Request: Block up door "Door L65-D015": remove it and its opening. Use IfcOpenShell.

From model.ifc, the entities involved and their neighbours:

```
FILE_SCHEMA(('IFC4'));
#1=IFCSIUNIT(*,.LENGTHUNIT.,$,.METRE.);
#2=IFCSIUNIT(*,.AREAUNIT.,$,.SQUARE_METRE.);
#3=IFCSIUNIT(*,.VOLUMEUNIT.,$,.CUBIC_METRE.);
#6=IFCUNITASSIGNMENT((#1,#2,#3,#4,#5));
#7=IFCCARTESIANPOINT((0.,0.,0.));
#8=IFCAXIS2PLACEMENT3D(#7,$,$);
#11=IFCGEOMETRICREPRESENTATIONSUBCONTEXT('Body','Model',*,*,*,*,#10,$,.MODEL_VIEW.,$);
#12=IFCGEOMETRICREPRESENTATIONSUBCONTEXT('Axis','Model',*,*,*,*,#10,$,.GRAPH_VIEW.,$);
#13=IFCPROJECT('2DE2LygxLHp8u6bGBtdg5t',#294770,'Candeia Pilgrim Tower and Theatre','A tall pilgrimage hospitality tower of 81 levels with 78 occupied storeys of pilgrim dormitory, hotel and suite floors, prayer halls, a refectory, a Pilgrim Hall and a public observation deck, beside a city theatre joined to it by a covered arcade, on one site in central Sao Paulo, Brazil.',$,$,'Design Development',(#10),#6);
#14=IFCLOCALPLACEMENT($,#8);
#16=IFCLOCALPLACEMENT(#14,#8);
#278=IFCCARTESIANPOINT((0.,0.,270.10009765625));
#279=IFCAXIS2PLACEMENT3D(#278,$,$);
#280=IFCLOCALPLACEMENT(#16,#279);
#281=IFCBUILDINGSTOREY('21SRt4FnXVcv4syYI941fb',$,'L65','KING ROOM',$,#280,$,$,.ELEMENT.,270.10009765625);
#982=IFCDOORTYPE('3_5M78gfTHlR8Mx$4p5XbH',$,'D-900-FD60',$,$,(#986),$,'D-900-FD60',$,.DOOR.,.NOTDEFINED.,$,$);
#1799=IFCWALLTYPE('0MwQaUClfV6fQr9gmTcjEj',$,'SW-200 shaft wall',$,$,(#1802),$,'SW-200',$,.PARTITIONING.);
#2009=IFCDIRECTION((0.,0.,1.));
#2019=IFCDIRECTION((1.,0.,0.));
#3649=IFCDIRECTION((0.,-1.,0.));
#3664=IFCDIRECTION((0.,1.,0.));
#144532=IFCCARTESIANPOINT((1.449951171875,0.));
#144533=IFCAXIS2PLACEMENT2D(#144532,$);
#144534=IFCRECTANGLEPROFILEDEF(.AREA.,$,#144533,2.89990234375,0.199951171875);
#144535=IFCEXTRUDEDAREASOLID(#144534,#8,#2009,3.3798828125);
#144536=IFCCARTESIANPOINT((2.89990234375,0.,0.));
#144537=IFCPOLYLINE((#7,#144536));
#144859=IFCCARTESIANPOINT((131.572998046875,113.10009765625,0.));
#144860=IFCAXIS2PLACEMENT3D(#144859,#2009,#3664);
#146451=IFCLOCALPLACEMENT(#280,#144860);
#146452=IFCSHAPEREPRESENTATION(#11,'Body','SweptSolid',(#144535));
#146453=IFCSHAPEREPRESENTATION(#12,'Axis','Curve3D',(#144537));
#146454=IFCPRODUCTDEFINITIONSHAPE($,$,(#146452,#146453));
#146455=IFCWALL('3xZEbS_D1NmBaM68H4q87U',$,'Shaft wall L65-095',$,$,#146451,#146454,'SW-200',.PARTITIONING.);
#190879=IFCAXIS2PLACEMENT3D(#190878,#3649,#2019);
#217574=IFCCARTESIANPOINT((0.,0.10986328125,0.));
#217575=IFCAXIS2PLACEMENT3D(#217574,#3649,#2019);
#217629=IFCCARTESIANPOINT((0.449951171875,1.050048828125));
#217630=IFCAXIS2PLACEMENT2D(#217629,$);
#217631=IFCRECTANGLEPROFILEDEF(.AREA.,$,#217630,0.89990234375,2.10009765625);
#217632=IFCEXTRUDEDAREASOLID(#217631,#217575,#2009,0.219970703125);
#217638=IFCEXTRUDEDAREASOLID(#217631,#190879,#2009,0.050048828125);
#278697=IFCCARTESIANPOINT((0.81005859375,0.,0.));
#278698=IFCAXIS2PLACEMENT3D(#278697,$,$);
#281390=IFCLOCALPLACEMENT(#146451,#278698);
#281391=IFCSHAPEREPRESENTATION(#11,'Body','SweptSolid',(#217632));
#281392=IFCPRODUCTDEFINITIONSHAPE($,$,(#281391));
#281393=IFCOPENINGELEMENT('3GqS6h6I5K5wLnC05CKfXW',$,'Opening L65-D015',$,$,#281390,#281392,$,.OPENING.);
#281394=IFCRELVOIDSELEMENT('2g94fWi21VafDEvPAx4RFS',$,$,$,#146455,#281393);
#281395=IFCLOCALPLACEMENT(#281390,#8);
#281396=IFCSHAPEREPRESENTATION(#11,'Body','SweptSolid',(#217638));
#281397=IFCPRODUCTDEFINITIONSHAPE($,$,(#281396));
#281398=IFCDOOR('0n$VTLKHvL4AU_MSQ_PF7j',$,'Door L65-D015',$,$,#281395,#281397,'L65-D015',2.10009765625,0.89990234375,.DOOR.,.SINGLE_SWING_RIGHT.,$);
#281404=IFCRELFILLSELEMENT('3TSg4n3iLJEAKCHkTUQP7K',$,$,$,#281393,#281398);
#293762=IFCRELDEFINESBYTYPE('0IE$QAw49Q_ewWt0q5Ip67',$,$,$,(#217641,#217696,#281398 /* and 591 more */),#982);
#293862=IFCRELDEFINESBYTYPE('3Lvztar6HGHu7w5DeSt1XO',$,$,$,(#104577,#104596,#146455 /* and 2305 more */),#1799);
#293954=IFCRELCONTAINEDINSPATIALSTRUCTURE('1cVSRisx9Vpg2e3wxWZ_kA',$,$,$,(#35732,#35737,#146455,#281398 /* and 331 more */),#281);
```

```python
import ifcopenshell
import ifcopenshell.api.feature
import ifcopenshell.api.root
import ifcopenshell.geom
import ifcopenshell.util.shape

model = ifcopenshell.open("model.ifc")
settings = ifcopenshell.geom.settings()


def volume(element):
    """Net volume in cubic metres, openings subtracted."""
    shape = ifcopenshell.geom.create_shape(settings, element)
    return ifcopenshell.util.shape.get_volume(shape.geometry)


door = model.by_guid("0n$VTLKHvL4AU_MSQ_PF7j")
opening = door.FillsVoids[0].RelatingOpeningElement
wall = opening.VoidsElements[0].RelatingBuildingElement
before = volume(wall)

ifcopenshell.api.root.remove_product(model, product=door)
ifcopenshell.api.feature.remove_feature(model, feature=opening)

after = volume(wall)

print(f"wall volume {before:.3f} -> {after:.3f} m3")

model.write("model_v2.ifc")
```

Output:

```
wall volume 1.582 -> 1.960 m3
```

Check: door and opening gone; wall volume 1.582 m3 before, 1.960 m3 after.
